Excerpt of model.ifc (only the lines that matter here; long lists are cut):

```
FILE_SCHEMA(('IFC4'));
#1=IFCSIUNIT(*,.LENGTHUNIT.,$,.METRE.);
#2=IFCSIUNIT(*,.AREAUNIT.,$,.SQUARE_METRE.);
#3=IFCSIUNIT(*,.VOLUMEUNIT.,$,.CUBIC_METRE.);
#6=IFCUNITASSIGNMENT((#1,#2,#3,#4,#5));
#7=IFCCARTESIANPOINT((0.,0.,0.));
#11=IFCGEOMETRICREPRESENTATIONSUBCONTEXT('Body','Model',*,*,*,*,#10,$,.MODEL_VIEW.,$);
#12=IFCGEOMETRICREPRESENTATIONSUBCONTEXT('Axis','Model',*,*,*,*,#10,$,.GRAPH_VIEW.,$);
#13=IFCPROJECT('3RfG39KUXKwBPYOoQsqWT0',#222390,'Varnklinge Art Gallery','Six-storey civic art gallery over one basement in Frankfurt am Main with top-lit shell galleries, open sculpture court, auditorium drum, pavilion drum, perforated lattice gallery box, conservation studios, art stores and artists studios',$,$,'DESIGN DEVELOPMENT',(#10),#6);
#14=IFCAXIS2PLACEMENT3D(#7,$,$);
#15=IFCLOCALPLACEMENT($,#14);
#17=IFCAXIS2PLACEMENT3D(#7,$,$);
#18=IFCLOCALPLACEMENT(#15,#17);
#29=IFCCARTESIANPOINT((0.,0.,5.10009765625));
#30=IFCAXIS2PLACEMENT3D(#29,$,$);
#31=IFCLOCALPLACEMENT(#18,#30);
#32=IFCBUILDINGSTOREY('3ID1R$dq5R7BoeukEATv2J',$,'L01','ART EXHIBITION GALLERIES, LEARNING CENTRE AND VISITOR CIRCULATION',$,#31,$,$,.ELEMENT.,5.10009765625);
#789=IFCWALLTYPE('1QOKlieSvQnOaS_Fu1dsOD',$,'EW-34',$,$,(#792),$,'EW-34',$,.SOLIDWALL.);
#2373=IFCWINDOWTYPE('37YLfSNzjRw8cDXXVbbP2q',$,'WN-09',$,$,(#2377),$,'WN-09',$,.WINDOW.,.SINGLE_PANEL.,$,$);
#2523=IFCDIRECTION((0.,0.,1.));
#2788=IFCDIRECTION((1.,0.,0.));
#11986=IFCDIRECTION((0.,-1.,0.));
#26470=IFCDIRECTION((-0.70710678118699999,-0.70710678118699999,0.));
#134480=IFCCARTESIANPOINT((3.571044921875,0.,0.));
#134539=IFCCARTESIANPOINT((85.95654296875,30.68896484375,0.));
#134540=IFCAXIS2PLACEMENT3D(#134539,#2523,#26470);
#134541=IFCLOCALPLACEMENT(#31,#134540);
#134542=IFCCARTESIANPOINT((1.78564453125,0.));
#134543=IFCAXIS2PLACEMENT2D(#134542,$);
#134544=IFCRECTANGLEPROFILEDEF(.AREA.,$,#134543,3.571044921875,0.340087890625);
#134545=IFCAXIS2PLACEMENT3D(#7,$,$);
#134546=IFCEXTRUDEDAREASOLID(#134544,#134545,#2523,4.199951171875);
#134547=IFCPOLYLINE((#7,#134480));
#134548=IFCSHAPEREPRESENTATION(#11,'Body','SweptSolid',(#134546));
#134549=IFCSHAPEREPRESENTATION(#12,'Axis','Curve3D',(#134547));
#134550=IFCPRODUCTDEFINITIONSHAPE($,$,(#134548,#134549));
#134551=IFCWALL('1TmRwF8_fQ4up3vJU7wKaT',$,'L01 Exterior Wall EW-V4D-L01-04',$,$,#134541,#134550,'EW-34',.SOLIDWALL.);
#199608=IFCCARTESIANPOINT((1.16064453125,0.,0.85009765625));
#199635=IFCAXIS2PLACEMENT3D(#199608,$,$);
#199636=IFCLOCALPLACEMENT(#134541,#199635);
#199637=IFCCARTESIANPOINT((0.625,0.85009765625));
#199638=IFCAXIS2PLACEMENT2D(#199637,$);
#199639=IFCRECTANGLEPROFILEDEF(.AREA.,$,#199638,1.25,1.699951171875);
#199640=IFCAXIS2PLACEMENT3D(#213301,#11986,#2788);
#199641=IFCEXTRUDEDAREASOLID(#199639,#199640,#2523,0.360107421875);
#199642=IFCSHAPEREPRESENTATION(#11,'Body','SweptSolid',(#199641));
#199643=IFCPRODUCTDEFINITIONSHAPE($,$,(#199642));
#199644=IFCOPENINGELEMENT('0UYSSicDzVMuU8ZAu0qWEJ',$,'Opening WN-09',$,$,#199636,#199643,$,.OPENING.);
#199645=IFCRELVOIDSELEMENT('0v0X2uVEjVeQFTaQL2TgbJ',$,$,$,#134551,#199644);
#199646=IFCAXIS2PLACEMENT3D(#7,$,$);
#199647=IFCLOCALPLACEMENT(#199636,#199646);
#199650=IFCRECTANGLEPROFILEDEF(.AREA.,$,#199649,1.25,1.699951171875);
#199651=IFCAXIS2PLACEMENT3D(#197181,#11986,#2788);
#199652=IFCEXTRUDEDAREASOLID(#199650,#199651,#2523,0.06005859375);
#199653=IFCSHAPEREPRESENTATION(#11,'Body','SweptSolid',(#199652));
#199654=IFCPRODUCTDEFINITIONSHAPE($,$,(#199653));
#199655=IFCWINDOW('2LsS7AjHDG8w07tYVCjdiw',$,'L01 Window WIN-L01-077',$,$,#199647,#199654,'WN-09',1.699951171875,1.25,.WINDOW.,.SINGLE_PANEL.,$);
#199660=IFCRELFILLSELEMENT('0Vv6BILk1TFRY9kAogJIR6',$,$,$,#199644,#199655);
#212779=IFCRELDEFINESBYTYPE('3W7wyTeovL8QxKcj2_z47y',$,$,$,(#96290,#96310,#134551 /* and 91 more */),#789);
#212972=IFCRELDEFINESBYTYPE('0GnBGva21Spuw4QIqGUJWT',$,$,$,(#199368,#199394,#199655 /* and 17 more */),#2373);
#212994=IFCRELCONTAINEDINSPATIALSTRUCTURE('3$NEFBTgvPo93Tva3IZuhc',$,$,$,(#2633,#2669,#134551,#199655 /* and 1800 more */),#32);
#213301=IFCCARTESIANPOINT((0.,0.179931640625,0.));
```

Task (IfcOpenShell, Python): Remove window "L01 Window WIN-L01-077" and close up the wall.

```python
import ifcopenshell
import ifcopenshell.api.feature
import ifcopenshell.api.root
import ifcopenshell.geom
import ifcopenshell.util.shape

model = ifcopenshell.open("model.ifc")
settings = ifcopenshell.geom.settings()


def volume(element):
    """Net volume in cubic metres, openings subtracted."""
    shape = ifcopenshell.geom.create_shape(settings, element)
    return ifcopenshell.util.shape.get_volume(shape.geometry)


window = model.by_guid("2LsS7AjHDG8w07tYVCjdiw")
opening = window.FillsVoids[0].RelatingOpeningElement
wall = opening.VoidsElements[0].RelatingBuildingElement
before = volume(wall)

ifcopenshell.api.root.remove_product(model, product=window)
ifcopenshell.api.feature.remove_feature(model, feature=opening)

after = volume(wall)

print(f"wall volume {before:.3f} -> {after:.3f} m3")

model.write("model_edited.ifc")
```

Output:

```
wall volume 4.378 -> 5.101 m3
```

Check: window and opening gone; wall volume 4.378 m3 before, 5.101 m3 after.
